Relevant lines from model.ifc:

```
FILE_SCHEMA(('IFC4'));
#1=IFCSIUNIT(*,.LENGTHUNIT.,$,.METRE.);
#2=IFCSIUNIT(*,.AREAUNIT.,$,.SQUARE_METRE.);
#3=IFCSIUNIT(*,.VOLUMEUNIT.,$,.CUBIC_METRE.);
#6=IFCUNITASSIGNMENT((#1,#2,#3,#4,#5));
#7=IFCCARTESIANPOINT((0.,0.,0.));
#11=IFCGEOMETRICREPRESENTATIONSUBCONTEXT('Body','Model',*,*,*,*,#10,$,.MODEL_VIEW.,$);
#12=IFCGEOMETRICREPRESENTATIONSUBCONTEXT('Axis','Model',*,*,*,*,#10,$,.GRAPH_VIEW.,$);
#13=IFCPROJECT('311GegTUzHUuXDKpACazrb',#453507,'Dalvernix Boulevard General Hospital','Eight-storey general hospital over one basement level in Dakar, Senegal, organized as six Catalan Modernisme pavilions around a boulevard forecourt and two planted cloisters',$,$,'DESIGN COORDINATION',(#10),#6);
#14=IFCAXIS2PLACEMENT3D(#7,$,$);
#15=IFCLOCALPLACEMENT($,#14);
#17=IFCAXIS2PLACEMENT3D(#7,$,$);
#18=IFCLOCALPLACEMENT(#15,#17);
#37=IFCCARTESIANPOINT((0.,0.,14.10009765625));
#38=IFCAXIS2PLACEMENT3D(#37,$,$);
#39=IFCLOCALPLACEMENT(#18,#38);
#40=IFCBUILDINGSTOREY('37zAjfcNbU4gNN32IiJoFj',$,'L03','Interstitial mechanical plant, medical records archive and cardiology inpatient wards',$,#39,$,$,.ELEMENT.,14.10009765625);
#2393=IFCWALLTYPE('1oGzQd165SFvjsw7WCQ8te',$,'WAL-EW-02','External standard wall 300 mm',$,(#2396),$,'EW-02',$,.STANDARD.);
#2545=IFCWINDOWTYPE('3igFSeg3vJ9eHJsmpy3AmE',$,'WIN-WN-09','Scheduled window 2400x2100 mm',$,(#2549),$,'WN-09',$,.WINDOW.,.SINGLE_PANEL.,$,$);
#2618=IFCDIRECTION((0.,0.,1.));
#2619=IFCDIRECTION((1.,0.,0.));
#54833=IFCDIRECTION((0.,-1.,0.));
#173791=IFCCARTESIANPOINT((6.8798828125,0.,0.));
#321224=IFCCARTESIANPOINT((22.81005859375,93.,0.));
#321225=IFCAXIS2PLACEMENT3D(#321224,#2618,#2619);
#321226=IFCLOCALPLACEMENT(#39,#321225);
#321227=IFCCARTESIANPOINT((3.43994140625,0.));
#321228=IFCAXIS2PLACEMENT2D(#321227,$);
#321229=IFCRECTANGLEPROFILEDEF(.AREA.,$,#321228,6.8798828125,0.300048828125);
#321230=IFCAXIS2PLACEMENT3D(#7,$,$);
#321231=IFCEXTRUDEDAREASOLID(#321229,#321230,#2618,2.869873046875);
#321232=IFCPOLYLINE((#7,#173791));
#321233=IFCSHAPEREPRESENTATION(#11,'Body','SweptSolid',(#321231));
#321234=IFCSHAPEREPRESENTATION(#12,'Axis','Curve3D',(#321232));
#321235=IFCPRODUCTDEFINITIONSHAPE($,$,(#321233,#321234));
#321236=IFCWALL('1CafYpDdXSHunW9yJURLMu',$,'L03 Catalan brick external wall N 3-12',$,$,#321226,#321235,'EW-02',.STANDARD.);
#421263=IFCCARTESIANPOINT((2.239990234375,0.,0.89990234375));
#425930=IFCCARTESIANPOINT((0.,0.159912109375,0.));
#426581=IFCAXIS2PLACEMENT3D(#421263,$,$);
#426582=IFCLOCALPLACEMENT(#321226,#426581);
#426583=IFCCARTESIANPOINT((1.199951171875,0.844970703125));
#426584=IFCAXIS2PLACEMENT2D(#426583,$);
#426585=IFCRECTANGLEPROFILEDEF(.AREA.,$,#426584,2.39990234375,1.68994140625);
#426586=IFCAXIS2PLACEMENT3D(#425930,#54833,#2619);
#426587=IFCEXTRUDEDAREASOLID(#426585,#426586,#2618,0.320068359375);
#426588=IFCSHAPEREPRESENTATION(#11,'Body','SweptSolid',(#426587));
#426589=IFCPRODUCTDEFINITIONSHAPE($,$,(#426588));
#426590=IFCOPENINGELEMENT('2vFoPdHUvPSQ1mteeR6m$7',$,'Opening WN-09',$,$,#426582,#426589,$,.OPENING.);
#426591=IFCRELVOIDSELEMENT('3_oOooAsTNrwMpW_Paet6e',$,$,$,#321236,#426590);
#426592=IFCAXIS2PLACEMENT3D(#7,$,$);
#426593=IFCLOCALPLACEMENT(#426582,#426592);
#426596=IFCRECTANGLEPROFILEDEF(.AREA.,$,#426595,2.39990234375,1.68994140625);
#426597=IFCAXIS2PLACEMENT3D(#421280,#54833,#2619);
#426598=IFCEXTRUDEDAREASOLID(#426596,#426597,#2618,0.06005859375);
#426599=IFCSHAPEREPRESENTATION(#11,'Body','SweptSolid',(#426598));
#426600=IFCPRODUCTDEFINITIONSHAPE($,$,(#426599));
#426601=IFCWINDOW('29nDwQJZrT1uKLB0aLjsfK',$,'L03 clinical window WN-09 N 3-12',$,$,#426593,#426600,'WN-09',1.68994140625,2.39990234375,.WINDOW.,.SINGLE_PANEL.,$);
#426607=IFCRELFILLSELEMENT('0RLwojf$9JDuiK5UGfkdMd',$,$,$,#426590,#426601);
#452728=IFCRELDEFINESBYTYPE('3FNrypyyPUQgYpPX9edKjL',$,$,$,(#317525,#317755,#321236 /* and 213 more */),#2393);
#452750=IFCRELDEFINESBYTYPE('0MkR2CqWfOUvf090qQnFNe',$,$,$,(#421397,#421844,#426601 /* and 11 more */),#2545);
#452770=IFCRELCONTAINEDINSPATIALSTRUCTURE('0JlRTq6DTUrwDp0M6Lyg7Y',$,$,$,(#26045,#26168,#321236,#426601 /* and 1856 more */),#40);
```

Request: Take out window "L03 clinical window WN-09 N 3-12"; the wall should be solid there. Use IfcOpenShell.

```python
import ifcopenshell
import ifcopenshell.api.feature
import ifcopenshell.api.root
import ifcopenshell.geom
import ifcopenshell.util.shape

model = ifcopenshell.open("model.ifc")
settings = ifcopenshell.geom.settings()


def volume(element):
    """Net volume in cubic metres, openings subtracted."""
    shape = ifcopenshell.geom.create_shape(settings, element)
    return ifcopenshell.util.shape.get_volume(shape.geometry)


window = model.by_id(426601)
opening = window.FillsVoids[0].RelatingOpeningElement
wall = opening.VoidsElements[0].RelatingBuildingElement
before = volume(wall)

ifcopenshell.api.root.remove_product(model, product=window)
ifcopenshell.api.feature.remove_feature(model, feature=opening)

after = volume(wall)

print(f"wall volume {before:.3f} -> {after:.3f} m3")

model.write("model_v2.ifc")
```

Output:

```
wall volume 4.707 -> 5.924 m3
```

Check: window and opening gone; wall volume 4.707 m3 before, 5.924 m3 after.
